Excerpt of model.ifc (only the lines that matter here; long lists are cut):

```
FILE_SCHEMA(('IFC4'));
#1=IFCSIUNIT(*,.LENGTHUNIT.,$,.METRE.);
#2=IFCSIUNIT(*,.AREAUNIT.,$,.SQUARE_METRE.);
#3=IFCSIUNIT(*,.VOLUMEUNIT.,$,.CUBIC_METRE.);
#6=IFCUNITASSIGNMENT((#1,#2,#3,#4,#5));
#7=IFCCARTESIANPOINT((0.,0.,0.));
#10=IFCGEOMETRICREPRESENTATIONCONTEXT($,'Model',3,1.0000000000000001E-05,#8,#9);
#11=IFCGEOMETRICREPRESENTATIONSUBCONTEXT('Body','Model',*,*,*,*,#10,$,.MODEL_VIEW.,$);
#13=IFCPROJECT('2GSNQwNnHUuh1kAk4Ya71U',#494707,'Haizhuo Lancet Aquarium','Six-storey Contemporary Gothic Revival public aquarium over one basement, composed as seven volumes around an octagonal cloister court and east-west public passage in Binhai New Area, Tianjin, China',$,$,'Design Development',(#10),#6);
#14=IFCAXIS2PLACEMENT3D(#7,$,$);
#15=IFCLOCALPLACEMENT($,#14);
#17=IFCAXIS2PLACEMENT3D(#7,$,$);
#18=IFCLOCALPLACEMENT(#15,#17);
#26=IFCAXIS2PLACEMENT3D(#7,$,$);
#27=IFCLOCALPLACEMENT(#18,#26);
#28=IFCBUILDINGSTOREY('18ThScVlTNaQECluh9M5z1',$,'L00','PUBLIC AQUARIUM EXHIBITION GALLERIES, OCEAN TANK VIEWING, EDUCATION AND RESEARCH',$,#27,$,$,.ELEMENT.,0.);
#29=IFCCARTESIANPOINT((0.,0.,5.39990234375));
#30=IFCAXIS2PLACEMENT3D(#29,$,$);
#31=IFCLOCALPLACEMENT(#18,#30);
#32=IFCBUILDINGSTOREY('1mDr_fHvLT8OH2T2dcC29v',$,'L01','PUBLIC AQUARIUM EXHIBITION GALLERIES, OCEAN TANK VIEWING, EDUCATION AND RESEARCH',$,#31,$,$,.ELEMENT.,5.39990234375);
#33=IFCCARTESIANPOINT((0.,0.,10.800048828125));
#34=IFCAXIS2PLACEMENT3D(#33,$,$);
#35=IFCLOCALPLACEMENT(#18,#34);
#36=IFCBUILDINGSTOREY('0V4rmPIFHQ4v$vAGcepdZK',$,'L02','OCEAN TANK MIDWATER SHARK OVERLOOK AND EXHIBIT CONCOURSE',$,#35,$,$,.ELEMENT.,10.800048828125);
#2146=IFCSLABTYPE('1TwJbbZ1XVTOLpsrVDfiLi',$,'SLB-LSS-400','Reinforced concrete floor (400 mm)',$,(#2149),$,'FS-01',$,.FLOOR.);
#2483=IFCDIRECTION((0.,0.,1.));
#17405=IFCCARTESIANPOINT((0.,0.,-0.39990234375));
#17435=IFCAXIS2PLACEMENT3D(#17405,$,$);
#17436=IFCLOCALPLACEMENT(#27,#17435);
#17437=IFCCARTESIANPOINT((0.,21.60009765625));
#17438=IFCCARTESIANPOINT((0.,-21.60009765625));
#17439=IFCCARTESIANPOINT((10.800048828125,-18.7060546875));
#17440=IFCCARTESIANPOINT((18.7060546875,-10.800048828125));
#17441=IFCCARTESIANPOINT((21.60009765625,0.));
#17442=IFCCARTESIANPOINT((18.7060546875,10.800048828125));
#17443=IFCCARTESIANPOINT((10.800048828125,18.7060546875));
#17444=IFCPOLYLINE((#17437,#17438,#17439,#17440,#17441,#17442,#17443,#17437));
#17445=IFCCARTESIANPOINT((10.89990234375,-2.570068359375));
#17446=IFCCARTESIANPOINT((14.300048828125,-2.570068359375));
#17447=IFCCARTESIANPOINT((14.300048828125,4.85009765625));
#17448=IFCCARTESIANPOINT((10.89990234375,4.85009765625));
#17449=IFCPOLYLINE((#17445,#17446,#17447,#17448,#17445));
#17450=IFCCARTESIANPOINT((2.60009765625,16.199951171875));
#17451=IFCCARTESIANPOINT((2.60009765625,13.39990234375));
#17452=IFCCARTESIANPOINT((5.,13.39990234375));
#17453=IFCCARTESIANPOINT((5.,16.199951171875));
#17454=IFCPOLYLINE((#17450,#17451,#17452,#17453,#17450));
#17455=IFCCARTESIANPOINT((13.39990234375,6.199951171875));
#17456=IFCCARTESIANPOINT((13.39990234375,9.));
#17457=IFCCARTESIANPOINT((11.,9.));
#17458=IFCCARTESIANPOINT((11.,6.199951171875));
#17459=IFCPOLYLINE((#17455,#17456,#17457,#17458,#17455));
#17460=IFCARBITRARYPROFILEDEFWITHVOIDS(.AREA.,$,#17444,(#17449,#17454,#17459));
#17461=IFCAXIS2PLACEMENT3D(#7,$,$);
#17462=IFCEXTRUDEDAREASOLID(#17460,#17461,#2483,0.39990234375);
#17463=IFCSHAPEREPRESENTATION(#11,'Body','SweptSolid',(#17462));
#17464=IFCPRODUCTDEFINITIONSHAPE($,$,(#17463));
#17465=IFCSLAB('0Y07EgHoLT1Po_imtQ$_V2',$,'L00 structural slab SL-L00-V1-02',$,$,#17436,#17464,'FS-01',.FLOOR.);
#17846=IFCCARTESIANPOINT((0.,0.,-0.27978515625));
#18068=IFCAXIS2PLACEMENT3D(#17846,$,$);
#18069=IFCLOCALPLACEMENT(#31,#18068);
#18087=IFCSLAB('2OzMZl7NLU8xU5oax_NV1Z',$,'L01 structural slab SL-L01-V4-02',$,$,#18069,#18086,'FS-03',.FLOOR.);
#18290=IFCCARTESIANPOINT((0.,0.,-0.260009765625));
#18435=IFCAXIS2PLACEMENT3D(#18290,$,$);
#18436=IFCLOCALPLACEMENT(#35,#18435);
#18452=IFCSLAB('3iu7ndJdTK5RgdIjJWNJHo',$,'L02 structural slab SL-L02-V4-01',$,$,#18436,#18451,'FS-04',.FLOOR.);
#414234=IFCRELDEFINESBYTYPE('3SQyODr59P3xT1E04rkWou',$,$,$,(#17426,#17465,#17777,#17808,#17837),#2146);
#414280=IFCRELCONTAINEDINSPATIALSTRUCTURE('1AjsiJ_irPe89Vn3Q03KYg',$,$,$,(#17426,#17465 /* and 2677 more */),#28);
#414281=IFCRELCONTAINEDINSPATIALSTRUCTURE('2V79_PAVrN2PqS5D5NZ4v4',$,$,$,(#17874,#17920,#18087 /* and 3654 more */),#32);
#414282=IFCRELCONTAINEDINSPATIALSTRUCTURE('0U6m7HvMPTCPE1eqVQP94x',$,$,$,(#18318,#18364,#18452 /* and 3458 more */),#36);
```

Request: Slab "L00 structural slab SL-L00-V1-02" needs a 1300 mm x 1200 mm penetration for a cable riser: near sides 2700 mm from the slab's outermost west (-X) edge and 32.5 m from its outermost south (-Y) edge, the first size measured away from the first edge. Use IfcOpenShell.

```python
import numpy as np
import ifcopenshell
import ifcopenshell.api.feature
import ifcopenshell.api.geometry
import ifcopenshell.api.root
import ifcopenshell.geom
import ifcopenshell.util.placement
import ifcopenshell.util.representation
import ifcopenshell.util.shape
import ifcopenshell.util.unit

model = ifcopenshell.open("model.ifc")
unit_scale = ifcopenshell.util.unit.calculate_unit_scale(model)
settings = ifcopenshell.geom.settings()


def volume(element):
    """Net volume in cubic metres, openings subtracted."""
    shape = ifcopenshell.geom.create_shape(settings, element)
    return ifcopenshell.util.shape.get_volume(shape.geometry)


slab = model.by_id(17465)
before = volume(slab)

# Extent in the slab's own axes, in metres. The edges named are its -X and -Y sides.
slab_shape = ifcopenshell.geom.create_shape(settings, slab)
vertices = ifcopenshell.util.shape.get_vertices(slab_shape.geometry)
x_min, y_min, bottom = vertices.min(axis=0)
top = vertices[:, 2].max()

opening = ifcopenshell.api.root.create_entity(model, ifc_class="IfcOpeningElement", name="Cable riser opening", predefined_type="OPENING")
context = ifcopenshell.util.representation.get_context(model, "Model", "Body", "MODEL_VIEW")
width, depth = 1.3, 1.2
outline = [(0.0, 0.0), (width, 0.0), (width, depth), (0.0, depth), (0.0, 0.0)]
# Overshoot both faces by 50 mm so the cut is clean.
shape = ifcopenshell.api.geometry.add_slab_representation(
    model, context=context, depth=top - bottom + 0.1, polyline=outline
)
ifcopenshell.api.geometry.assign_representation(model, product=opening, representation=shape)

matrix = ifcopenshell.util.placement.get_local_placement(slab.ObjectPlacement)
matrix[:, 3] = matrix @ np.append(np.array([x_min + 2.7, y_min + 32.5, bottom - 0.05]) / unit_scale, 1.0)
ifcopenshell.api.geometry.edit_object_placement(model, product=opening, matrix=matrix, is_si=False)
ifcopenshell.api.feature.add_feature(model, feature=opening, element=slab)

after = volume(slab)

print(f"slab volume {before:.3f} -> {after:.3f} m3")

model.write("model-out.ifc")
```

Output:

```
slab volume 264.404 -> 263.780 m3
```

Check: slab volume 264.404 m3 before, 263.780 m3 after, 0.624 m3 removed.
